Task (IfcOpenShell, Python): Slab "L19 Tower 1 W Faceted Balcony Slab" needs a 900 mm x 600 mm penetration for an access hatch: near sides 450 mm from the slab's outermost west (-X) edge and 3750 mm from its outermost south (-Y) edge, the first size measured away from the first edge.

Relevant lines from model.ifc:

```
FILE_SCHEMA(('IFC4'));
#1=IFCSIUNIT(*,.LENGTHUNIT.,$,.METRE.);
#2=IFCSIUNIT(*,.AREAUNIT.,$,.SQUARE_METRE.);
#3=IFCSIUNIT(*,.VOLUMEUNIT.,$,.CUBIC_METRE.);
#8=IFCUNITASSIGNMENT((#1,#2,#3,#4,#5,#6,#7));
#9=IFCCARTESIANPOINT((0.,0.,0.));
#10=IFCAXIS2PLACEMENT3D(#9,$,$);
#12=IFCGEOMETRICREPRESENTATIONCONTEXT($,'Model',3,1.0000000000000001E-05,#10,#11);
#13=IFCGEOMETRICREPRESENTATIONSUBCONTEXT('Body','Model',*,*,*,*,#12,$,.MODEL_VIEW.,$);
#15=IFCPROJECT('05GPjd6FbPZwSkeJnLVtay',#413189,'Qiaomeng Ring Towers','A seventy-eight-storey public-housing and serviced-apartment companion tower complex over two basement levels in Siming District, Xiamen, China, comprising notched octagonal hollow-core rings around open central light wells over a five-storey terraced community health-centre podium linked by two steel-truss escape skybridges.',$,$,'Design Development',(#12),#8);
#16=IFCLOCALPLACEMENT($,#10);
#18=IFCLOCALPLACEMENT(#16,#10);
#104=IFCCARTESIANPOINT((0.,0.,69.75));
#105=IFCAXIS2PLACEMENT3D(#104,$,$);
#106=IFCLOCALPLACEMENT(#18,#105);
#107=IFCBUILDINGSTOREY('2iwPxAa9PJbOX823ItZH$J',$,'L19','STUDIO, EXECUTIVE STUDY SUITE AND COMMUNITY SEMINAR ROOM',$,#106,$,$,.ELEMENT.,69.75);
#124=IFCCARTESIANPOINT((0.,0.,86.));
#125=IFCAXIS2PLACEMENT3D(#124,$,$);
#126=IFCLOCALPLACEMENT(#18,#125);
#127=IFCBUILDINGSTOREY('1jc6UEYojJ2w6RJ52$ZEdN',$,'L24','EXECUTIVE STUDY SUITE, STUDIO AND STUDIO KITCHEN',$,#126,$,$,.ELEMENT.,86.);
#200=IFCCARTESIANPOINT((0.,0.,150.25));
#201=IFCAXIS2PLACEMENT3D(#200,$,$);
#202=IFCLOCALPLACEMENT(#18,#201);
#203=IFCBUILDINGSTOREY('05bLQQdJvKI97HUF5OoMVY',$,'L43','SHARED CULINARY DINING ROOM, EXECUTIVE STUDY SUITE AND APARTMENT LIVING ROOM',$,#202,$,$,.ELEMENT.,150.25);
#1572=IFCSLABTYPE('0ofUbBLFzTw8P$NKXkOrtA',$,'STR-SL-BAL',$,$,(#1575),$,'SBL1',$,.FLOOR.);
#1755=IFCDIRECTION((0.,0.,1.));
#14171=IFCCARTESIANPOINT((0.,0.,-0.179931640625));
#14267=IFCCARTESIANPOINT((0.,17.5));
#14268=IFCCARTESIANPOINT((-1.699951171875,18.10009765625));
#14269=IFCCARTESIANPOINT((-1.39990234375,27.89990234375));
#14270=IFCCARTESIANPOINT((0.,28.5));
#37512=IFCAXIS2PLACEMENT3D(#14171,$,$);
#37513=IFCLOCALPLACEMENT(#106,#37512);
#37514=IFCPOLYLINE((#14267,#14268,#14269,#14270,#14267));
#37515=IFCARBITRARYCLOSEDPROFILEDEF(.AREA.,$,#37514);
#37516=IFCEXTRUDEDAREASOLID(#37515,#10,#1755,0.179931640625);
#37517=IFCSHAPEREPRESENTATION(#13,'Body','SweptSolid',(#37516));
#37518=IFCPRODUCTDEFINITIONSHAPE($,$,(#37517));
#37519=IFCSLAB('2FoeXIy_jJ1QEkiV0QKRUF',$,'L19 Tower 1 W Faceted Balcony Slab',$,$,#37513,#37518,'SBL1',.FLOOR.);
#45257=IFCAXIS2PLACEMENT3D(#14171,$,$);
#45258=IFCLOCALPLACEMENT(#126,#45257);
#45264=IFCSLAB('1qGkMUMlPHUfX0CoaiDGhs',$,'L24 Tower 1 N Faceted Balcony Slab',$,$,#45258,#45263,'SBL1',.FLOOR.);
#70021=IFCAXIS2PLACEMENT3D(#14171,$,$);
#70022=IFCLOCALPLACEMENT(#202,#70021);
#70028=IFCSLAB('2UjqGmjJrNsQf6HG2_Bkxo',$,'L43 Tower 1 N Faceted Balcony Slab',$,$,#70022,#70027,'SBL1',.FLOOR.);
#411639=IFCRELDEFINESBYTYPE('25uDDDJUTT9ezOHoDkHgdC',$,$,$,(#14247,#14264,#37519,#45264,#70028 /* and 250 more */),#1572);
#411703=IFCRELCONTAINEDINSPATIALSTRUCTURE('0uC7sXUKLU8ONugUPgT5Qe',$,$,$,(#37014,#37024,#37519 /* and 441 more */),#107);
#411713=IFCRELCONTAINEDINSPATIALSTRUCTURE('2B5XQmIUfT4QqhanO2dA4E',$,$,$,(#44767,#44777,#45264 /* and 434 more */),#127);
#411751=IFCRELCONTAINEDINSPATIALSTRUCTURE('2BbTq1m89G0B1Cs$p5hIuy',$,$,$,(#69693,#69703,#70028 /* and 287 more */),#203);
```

```python
import numpy as np
import ifcopenshell
import ifcopenshell.api.feature
import ifcopenshell.api.geometry
import ifcopenshell.api.root
import ifcopenshell.geom
import ifcopenshell.util.placement
import ifcopenshell.util.representation
import ifcopenshell.util.shape
import ifcopenshell.util.unit

model = ifcopenshell.open("model.ifc")
unit_scale = ifcopenshell.util.unit.calculate_unit_scale(model)
settings = ifcopenshell.geom.settings()


def volume(element):
    """Net volume in cubic metres, openings subtracted."""
    shape = ifcopenshell.geom.create_shape(settings, element)
    return ifcopenshell.util.shape.get_volume(shape.geometry)


slab = model.by_id(37519)
before = volume(slab)

# Extent in the slab's own axes, in metres. The edges named are its -X and -Y sides.
slab_shape = ifcopenshell.geom.create_shape(settings, slab)
vertices = ifcopenshell.util.shape.get_vertices(slab_shape.geometry)
x_min, y_min, bottom = vertices.min(axis=0)
top = vertices[:, 2].max()

opening = ifcopenshell.api.root.create_entity(model, ifc_class="IfcOpeningElement", name="Access hatch opening", predefined_type="OPENING")
context = ifcopenshell.util.representation.get_context(model, "Model", "Body", "MODEL_VIEW")
width, depth = 0.9, 0.6
outline = [(0.0, 0.0), (width, 0.0), (width, depth), (0.0, depth), (0.0, 0.0)]
# Overshoot both faces by 50 mm so the cut is clean.
shape = ifcopenshell.api.geometry.add_slab_representation(
    model, context=context, depth=top - bottom + 0.1, polyline=outline
)
ifcopenshell.api.geometry.assign_representation(model, product=opening, representation=shape)

matrix = ifcopenshell.util.placement.get_local_placement(slab.ObjectPlacement)
matrix[:, 3] = matrix @ np.append(np.array([x_min + 0.45, y_min + 3.75, bottom - 0.05]) / unit_scale, 1.0)
ifcopenshell.api.geometry.edit_object_placement(model, product=opening, matrix=matrix, is_si=False)
ifcopenshell.api.feature.add_feature(model, feature=opening, element=slab)

after = volume(slab)

print(f"slab volume {before:.3f} -> {after:.3f} m3")

model.write("model_rev.ifc")
```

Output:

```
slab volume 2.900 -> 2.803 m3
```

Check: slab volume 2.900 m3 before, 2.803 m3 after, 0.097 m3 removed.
